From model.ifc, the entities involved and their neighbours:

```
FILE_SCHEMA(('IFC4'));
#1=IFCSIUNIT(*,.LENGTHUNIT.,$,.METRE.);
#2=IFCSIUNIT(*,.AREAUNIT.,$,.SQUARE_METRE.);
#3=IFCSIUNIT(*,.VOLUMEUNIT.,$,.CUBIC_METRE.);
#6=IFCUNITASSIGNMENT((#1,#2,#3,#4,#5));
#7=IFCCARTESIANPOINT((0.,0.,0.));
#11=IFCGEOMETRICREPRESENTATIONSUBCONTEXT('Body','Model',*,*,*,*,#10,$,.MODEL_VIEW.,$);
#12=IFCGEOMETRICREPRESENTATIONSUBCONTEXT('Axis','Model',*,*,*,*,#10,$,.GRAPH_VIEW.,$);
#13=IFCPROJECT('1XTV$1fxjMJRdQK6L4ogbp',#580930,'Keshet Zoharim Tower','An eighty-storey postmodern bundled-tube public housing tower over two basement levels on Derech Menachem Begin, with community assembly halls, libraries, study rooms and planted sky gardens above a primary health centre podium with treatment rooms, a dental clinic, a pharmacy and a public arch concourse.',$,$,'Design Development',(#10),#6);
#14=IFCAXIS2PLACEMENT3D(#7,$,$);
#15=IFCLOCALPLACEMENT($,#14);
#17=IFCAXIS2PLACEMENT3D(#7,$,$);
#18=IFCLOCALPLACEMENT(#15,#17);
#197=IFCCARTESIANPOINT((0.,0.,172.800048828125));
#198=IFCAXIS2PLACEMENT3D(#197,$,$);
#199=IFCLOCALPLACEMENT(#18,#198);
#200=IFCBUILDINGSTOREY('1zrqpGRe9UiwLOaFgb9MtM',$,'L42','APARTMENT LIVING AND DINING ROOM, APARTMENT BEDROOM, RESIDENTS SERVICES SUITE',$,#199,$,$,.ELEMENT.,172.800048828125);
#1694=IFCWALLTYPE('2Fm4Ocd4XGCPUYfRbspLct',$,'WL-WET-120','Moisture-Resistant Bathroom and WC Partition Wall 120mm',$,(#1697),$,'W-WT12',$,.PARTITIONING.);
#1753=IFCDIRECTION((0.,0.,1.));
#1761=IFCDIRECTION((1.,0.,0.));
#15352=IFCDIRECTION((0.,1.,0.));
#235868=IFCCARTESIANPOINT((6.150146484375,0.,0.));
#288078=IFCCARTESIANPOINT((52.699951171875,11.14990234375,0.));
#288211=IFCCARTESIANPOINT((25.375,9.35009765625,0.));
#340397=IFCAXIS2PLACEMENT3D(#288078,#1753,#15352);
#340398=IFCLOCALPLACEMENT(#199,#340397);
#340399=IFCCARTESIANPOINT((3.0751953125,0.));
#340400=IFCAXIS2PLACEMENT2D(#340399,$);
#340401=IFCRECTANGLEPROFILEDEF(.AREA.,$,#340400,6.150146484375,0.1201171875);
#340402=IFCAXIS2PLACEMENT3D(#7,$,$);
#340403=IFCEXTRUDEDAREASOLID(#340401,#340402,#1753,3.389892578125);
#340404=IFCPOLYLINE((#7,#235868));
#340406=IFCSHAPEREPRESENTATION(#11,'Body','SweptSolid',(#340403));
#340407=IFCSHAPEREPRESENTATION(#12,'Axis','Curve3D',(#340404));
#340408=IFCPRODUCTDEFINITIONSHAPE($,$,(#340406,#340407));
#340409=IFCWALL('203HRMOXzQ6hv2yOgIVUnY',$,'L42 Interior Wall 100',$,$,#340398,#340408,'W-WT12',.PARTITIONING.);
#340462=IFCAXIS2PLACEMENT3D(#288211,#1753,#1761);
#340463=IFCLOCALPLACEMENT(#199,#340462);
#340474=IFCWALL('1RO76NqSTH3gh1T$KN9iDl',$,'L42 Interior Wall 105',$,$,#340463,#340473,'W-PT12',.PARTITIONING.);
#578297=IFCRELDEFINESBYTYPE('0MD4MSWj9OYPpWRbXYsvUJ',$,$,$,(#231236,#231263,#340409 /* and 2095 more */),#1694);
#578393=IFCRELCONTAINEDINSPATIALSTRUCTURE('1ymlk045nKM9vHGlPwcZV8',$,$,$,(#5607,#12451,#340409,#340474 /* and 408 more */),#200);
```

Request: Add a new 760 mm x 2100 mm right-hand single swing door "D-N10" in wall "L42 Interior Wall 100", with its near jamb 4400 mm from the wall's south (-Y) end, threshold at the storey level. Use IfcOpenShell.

```python
import numpy as np
import ifcopenshell
import ifcopenshell.api.feature
import ifcopenshell.api.geometry
import ifcopenshell.api.root
import ifcopenshell.api.spatial
import ifcopenshell.geom
import ifcopenshell.util.element
import ifcopenshell.util.placement
import ifcopenshell.util.representation
import ifcopenshell.util.shape
import ifcopenshell.util.unit

model = ifcopenshell.open("model.ifc")
unit_scale = ifcopenshell.util.unit.calculate_unit_scale(model)
settings = ifcopenshell.geom.settings()


def volume(element):
    """Net volume in cubic metres, openings subtracted."""
    shape = ifcopenshell.geom.create_shape(settings, element)
    return ifcopenshell.util.shape.get_volume(shape.geometry)


wall = model.by_guid("203HRMOXzQ6hv2yOgIVUnY")
storey = ifcopenshell.util.element.get_container(wall, ifc_class="IfcBuildingStorey")
context = ifcopenshell.util.representation.get_context(model, "Model", "Body", "MODEL_VIEW")
before = volume(wall)

width, height, from_end, sill = 0.76, 2.1, 4.4, 0.0  # metres

# The wall runs along its own X axis, and the end named is its -X end.
wall_shape = ifcopenshell.geom.create_shape(settings, wall)
x, y, z = ifcopenshell.util.shape.get_vertices(wall_shape.geometry).T
start = x.min() + from_end
face, thickness = float(y.min()), float(y.max() - y.min())
wall_matrix = ifcopenshell.util.placement.get_local_placement(wall.ObjectPlacement)
level = ifcopenshell.util.placement.get_local_placement(storey.ObjectPlacement)[2, 3]


def in_wall(x, y):
    """Placement at x, y metres in the wall's axes, at sill height."""
    matrix = wall_matrix.copy()
    matrix[:, 3] = wall_matrix @ np.array([x / unit_scale, y / unit_scale, 0.0, 1.0])
    matrix[2, 3] = level + sill / unit_scale
    return matrix


# Opening: a box that overshoots both wall faces by 50 mm.
opening = ifcopenshell.api.root.create_entity(model, ifc_class="IfcOpeningElement", predefined_type="OPENING")
box = ifcopenshell.api.geometry.add_wall_representation(
    model, context=context, length=width, height=height, thickness=thickness + 0.1
)
ifcopenshell.api.geometry.assign_representation(model, product=opening, representation=box)
ifcopenshell.api.geometry.edit_object_placement(model, product=opening, matrix=in_wall(start, face - 0.05), is_si=False)
ifcopenshell.api.feature.add_feature(model, feature=opening, element=wall)

door = ifcopenshell.api.root.create_entity(model, ifc_class="IfcDoor", name="D-N10", predefined_type="DOOR")
door.OverallWidth, door.OverallHeight = width / unit_scale, height / unit_scale
door.OperationType = "SINGLE_SWING_RIGHT"
body = ifcopenshell.api.geometry.add_door_representation(
    model,
    context=context,
    overall_width=door.OverallWidth,
    overall_height=door.OverallHeight,
    operation_type="SINGLE_SWING_RIGHT",
    lining_properties={"LiningDepth": thickness / unit_scale, "ThresholdDepth": thickness / unit_scale},
)
ifcopenshell.api.geometry.assign_representation(model, product=door, representation=body)
ifcopenshell.api.spatial.assign_container(model, products=[door], relating_structure=storey)
ifcopenshell.api.feature.add_filling(model, opening=opening, element=door)

# The lining spans the wall, so the door starts at the wall face.
ifcopenshell.api.geometry.edit_object_placement(model, product=door, matrix=in_wall(start, face), is_si=False)

after = volume(wall)

print(f"wall volume {before:.3f} -> {after:.3f} m3")

model.write("model_edited.ifc")
```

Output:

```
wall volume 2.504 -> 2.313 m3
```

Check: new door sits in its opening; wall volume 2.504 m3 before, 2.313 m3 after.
